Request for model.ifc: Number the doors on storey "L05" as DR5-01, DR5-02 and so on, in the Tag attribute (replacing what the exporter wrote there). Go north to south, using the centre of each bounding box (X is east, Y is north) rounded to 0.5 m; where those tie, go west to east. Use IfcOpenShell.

First a look at what the model holds.

```python
import ifcopenshell
import ifcopenshell.util.element
import ifcopenshell.util.placement

model = ifcopenshell.open("model.ifc")
print(model.schema)
storey = next(s for s in model.by_type("IfcBuildingStorey") if s.Name == "L05")
doors = [e for e in ifcopenshell.util.element.get_decomposition(storey) if e.is_a("IfcDoor")]
for e in sorted(doors, key=lambda e: e.id()):
    origin = ifcopenshell.util.placement.get_local_placement(e.ObjectPlacement)[:3, 3]
    print(e.id(), e.Tag, e.Name, origin.round(2) + 0.0, sep=" | ")
```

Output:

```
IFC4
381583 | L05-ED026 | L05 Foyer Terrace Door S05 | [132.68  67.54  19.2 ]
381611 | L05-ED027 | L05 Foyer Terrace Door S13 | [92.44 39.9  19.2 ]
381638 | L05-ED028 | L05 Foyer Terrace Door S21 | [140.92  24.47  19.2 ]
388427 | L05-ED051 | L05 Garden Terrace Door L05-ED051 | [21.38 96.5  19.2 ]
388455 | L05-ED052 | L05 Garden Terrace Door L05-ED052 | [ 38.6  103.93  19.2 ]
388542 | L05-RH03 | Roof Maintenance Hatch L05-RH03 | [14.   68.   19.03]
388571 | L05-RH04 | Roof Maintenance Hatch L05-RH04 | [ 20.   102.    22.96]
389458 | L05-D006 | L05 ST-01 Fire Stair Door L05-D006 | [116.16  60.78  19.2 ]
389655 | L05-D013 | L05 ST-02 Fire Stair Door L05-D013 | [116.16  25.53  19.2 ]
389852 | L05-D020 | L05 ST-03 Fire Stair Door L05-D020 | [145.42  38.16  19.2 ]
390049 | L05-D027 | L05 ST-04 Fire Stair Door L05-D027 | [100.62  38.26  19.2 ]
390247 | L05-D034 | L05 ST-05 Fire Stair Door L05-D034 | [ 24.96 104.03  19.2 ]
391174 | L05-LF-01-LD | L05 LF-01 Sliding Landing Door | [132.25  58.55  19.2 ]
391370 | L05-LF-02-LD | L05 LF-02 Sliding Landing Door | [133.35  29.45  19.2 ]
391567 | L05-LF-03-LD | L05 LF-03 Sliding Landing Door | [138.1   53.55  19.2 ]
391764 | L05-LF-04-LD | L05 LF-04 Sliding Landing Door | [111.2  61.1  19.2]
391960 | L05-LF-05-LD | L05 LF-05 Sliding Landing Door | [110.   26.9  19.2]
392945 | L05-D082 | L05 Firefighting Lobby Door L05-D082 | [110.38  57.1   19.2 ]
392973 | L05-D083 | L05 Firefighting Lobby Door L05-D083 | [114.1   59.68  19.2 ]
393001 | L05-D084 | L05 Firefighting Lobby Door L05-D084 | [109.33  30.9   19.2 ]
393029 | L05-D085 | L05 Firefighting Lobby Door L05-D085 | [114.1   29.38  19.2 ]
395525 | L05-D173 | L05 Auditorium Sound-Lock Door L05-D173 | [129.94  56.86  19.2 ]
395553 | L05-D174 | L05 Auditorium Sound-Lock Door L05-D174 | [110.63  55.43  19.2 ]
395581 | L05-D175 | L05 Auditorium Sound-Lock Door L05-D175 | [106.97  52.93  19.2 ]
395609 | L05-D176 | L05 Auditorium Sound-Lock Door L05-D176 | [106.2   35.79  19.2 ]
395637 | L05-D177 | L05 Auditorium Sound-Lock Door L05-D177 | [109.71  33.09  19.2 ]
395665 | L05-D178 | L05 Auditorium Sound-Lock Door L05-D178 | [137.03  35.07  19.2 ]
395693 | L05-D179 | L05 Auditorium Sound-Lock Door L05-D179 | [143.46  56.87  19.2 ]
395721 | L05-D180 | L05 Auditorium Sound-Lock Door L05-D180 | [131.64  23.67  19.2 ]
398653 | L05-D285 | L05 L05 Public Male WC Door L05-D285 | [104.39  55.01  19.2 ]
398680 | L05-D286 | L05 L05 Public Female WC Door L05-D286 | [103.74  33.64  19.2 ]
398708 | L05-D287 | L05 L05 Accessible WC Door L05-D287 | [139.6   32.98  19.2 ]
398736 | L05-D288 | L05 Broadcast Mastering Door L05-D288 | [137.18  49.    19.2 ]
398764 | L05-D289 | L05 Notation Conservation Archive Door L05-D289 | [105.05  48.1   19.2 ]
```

```python
import ifcopenshell
import ifcopenshell.geom
import ifcopenshell.util.element
import ifcopenshell.util.shape

model = ifcopenshell.open("model.ifc")
settings = ifcopenshell.geom.settings()
settings.set("use-world-coords", True)


def centre(element):
    shape = ifcopenshell.geom.create_shape(settings, element)
    return ifcopenshell.util.shape.get_bbox_centroid(shape.geometry)


storey = next(s for s in model.by_type("IfcBuildingStorey") if s.Name == "L05")
doors = [e for e in ifcopenshell.util.element.get_decomposition(storey) if e.is_a("IfcDoor")]

# Insertion points can sit at a corner or the storey origin, so sort by the geometry (in metres).
centres = {e: centre(e) for e in doors}
doors.sort(key=lambda e: (-round(centres[e][1] / 0.5), centres[e][0]))

for i, e in enumerate(doors, start=1):
    number = f"DR5-{i:02d}"
    e.Tag = number
    print(e.id(), number)

model.write("model_updated.ifc")
```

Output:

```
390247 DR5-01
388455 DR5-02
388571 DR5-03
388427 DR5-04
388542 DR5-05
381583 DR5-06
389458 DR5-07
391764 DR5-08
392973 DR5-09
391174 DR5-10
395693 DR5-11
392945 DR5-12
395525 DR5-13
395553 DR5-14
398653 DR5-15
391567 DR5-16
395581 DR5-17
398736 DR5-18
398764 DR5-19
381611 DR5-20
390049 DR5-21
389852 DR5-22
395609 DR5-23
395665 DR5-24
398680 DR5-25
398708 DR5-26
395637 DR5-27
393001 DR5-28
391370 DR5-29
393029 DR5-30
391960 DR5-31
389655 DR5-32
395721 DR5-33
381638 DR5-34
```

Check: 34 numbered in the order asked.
